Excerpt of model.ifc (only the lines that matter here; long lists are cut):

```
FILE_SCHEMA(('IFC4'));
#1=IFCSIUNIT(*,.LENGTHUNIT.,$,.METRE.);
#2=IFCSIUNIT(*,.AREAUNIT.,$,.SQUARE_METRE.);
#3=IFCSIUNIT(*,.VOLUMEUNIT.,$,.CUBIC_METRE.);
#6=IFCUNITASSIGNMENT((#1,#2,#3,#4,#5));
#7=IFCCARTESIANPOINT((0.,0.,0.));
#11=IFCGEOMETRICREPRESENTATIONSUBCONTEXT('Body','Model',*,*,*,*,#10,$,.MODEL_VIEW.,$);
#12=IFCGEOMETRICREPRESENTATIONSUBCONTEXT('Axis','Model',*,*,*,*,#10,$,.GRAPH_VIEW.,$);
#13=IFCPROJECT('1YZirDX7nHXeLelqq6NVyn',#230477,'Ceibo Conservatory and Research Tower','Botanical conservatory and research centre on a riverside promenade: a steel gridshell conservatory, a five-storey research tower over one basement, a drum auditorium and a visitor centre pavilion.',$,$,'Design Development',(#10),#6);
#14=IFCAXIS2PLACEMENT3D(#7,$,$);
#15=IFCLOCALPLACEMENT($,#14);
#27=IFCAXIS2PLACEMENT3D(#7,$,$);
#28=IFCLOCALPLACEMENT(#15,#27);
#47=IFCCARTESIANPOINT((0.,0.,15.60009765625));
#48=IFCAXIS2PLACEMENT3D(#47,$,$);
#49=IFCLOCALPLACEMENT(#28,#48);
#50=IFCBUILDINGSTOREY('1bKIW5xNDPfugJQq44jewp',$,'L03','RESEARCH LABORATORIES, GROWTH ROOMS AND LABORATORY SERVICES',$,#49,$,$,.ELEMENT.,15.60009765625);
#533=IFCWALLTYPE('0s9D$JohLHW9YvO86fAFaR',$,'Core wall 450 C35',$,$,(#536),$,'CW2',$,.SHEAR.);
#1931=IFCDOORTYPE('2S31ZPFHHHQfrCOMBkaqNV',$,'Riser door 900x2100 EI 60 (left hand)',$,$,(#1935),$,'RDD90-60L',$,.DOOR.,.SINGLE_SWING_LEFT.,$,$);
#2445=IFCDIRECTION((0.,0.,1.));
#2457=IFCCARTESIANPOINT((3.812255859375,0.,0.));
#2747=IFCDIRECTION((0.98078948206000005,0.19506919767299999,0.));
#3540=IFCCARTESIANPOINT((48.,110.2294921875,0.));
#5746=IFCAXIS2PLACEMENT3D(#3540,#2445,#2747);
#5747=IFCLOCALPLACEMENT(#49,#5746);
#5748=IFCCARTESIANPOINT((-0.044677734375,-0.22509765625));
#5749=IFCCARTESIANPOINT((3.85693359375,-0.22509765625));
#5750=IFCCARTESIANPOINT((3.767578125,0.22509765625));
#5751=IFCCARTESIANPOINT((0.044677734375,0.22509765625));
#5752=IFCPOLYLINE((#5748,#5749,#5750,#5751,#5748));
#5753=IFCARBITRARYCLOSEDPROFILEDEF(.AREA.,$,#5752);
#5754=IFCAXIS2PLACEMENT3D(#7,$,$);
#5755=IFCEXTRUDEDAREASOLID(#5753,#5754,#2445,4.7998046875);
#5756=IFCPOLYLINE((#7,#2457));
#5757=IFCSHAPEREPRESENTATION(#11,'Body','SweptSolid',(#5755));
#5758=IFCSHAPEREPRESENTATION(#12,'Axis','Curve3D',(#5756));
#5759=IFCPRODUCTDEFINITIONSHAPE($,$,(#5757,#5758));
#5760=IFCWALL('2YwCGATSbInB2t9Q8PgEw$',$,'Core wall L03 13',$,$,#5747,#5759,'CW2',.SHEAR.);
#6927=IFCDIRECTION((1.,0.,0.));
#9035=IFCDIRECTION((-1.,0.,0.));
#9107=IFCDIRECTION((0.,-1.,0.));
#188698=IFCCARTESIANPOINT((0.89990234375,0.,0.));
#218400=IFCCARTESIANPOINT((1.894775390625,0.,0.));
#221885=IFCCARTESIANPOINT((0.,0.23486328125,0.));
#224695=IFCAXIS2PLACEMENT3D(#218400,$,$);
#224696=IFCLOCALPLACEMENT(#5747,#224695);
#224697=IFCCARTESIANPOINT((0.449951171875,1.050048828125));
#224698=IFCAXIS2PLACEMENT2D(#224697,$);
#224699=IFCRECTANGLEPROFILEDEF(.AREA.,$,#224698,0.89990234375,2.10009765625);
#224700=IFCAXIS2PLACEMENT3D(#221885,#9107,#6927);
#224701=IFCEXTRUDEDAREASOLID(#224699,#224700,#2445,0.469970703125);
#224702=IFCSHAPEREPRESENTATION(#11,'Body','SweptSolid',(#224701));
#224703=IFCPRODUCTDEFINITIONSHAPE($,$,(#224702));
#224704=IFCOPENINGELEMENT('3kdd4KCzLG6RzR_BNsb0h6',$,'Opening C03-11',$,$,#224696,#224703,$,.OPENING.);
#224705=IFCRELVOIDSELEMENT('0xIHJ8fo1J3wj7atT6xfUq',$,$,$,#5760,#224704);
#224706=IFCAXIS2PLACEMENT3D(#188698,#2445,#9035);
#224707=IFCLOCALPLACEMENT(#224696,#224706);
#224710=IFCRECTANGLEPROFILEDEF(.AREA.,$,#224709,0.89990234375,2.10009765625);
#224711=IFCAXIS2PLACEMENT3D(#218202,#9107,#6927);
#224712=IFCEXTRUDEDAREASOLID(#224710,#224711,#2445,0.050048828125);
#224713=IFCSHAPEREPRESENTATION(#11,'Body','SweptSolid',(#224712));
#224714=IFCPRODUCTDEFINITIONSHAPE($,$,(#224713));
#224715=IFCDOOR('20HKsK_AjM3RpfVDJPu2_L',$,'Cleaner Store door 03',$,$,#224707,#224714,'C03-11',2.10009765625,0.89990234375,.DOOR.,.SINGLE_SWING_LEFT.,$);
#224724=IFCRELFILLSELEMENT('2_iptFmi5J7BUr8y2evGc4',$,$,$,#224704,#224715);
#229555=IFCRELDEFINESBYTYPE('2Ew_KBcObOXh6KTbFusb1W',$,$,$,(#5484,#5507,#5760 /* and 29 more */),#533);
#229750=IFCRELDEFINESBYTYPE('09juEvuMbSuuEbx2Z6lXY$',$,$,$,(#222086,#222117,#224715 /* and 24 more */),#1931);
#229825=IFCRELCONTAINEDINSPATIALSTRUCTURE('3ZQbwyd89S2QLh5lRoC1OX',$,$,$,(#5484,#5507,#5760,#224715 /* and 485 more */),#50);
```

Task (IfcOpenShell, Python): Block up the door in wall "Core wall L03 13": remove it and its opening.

```python
import ifcopenshell
import ifcopenshell.api.feature
import ifcopenshell.api.root
import ifcopenshell.geom
import ifcopenshell.util.shape

model = ifcopenshell.open("model.ifc")
settings = ifcopenshell.geom.settings()


def volume(element):
    """Net volume in cubic metres, openings subtracted."""
    shape = ifcopenshell.geom.create_shape(settings, element)
    return ifcopenshell.util.shape.get_volume(shape.geometry)


door = model.by_guid("20HKsK_AjM3RpfVDJPu2_L")
opening = door.FillsVoids[0].RelatingOpeningElement
wall = opening.VoidsElements[0].RelatingBuildingElement
before = volume(wall)

ifcopenshell.api.root.remove_product(model, product=door)
ifcopenshell.api.feature.remove_feature(model, feature=opening)

after = volume(wall)

print(f"wall volume {before:.3f} -> {after:.3f} m3")

model.write("model_rev.ifc")
```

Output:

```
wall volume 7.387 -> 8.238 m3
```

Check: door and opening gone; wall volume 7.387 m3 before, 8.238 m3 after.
